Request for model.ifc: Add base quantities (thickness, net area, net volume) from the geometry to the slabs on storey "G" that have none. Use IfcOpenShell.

First a look at what the model holds.

```python
import ifcopenshell
import ifcopenshell.util.element
import ifcopenshell.util.unit

model = ifcopenshell.open("model.ifc")
print(model.schema)
for unit_type in ("LENGTHUNIT", "AREAUNIT", "VOLUMEUNIT"):
    print(unit_type, ifcopenshell.util.unit.calculate_unit_scale(model, unit_type))
storey = next(s for s in model.by_type("IfcBuildingStorey") if s.Name == "G")
slabs = [e for e in ifcopenshell.util.element.get_decomposition(storey) if e.is_a("IfcSlab")]
for e in sorted(slabs, key=lambda e: e.id()):
    print(e.id(), e.is_a(), e.Name, list(ifcopenshell.util.element.get_psets(e, qtos_only=True)), sep=" | ")
```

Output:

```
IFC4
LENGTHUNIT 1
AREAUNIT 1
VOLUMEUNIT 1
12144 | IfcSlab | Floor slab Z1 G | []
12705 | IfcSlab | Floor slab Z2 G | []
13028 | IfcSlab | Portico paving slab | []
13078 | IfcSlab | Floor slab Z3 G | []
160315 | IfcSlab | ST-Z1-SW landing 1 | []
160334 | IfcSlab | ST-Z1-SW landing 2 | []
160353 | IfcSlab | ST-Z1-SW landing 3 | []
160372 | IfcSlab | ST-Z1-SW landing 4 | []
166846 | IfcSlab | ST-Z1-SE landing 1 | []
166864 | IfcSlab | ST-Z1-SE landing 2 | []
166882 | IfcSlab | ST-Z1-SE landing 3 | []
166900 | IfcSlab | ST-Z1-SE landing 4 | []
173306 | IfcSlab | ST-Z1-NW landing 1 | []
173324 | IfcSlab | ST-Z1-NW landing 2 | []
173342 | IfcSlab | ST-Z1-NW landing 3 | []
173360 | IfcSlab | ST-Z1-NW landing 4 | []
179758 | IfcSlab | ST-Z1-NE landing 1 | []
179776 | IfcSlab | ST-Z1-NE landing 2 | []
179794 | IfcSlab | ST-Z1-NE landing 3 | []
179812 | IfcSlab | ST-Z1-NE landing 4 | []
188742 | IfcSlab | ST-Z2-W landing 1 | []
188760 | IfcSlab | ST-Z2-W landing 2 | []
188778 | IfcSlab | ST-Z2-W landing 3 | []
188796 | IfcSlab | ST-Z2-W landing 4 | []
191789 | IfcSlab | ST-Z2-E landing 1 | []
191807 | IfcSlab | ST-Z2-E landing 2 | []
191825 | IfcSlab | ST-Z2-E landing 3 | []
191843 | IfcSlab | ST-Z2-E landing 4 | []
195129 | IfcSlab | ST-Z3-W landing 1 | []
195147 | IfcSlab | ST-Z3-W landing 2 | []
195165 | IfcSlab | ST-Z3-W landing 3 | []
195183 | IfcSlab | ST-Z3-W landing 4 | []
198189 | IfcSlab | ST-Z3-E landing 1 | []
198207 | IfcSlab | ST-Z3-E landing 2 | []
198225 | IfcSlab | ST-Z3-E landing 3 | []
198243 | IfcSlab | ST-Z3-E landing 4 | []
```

```python
import ifcopenshell
import ifcopenshell.api.pset
import ifcopenshell.geom
import ifcopenshell.util.element
import ifcopenshell.util.shape
import ifcopenshell.util.unit

model = ifcopenshell.open("model.ifc")
unit_scale = ifcopenshell.util.unit.calculate_unit_scale(model)
area_scale = ifcopenshell.util.unit.calculate_unit_scale(model, "AREAUNIT")
volume_scale = ifcopenshell.util.unit.calculate_unit_scale(model, "VOLUMEUNIT")
settings = ifcopenshell.geom.settings()

storey = next(s for s in model.by_type("IfcBuildingStorey") if s.Name == "G")
slabs = [e for e in ifcopenshell.util.element.get_decomposition(storey) if e.is_a("IfcSlab")]

for e in sorted(slabs, key=lambda e: e.id()):
    if ifcopenshell.util.element.get_psets(e, qtos_only=True, should_inherit=False):
        continue
    # Geometry comes back in metres, in the element's own axes.
    shape = ifcopenshell.geom.create_shape(settings, e)
    values = {
        "Width": ifcopenshell.util.shape.get_z(shape.geometry) / unit_scale,
        "NetArea": ifcopenshell.util.shape.get_footprint_area(shape.geometry) / area_scale,
        "NetVolume": ifcopenshell.util.shape.get_volume(shape.geometry) / volume_scale,
    }
    qto = ifcopenshell.api.pset.add_qto(model, product=e, name="Qto_SlabBaseQuantities")
    ifcopenshell.api.pset.edit_qto(model, qto=qto, properties=values)
    print(e.id(), {k: round(v, 3) for k, v in values.items()})

model.write("model_v2.ifc")
```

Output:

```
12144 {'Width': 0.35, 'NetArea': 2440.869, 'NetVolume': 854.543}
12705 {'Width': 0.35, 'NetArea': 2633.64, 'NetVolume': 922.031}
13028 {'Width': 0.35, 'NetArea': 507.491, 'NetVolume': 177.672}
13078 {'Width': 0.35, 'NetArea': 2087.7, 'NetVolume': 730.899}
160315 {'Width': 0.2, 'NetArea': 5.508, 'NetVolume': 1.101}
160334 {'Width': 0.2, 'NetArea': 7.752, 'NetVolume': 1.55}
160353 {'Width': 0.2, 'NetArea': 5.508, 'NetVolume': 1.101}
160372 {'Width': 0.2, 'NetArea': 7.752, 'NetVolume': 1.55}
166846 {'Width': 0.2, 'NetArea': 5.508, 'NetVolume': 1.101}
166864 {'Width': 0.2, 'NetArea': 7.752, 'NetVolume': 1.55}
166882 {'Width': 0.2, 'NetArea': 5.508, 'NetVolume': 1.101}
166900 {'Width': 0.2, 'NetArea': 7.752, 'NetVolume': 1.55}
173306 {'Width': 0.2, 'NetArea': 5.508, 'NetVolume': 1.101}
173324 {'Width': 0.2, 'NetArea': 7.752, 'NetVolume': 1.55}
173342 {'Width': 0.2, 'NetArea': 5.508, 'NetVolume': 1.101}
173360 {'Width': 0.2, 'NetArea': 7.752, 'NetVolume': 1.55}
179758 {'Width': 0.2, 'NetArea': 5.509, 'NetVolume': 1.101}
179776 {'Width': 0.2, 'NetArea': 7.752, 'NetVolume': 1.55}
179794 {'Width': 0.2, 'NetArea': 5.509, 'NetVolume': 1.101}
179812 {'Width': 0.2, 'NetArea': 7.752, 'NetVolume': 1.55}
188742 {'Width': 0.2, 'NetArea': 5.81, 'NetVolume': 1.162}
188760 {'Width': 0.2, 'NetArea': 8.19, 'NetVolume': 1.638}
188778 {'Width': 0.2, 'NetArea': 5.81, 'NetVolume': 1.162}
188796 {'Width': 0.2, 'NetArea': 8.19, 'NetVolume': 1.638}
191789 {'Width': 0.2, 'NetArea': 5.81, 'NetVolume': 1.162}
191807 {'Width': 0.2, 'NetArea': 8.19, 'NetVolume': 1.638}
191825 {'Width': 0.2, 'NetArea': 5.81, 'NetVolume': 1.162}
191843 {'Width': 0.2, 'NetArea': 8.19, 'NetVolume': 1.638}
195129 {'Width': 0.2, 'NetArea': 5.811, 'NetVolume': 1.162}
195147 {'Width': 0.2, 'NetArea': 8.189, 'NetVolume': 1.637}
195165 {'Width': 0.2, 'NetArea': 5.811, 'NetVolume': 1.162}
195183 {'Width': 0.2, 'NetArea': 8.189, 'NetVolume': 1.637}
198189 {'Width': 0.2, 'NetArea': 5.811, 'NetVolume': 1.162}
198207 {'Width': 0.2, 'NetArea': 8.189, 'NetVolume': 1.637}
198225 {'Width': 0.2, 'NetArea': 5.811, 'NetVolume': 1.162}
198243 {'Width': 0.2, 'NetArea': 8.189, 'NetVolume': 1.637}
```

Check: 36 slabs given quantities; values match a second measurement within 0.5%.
